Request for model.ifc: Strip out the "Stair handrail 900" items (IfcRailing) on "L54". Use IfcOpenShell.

First a look at what the model holds.

```python
import ifcopenshell
import ifcopenshell.util.element

model = ifcopenshell.open("model.ifc")
print(model.schema)
storey = next(s for s in model.by_type("IfcBuildingStorey") if s.Name == "L54")
railings = [e for e in ifcopenshell.util.element.get_decomposition(storey) if e.is_a("IfcRailing")]
seen = {}
for e in railings:
    element_type = ifcopenshell.util.element.get_type(e)
    name = element_type.Name if element_type not in (None, e) else None
    seen[name] = seen.get(name, 0) + 1
for name, count in sorted(seen.items(), key=str):
    print(count, "x", name)
```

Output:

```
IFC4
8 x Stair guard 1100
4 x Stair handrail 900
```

```python
import ifcopenshell
import ifcopenshell.api.root
import ifcopenshell.util.element

model = ifcopenshell.open("model.ifc")

storey = next(s for s in model.by_type("IfcBuildingStorey") if s.Name == "L54")
railings = [e for e in ifcopenshell.util.element.get_decomposition(storey) if e.is_a("IfcRailing")]
targets = [e for e in railings if (t := ifcopenshell.util.element.get_type(e)) not in (None, e) and t.Name == "Stair handrail 900"]

for e in targets:
    ifcopenshell.api.root.remove_product(model, product=e)
print(len(targets), "removed")

model.write("model-out.ifc")
```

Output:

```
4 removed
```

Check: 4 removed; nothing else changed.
